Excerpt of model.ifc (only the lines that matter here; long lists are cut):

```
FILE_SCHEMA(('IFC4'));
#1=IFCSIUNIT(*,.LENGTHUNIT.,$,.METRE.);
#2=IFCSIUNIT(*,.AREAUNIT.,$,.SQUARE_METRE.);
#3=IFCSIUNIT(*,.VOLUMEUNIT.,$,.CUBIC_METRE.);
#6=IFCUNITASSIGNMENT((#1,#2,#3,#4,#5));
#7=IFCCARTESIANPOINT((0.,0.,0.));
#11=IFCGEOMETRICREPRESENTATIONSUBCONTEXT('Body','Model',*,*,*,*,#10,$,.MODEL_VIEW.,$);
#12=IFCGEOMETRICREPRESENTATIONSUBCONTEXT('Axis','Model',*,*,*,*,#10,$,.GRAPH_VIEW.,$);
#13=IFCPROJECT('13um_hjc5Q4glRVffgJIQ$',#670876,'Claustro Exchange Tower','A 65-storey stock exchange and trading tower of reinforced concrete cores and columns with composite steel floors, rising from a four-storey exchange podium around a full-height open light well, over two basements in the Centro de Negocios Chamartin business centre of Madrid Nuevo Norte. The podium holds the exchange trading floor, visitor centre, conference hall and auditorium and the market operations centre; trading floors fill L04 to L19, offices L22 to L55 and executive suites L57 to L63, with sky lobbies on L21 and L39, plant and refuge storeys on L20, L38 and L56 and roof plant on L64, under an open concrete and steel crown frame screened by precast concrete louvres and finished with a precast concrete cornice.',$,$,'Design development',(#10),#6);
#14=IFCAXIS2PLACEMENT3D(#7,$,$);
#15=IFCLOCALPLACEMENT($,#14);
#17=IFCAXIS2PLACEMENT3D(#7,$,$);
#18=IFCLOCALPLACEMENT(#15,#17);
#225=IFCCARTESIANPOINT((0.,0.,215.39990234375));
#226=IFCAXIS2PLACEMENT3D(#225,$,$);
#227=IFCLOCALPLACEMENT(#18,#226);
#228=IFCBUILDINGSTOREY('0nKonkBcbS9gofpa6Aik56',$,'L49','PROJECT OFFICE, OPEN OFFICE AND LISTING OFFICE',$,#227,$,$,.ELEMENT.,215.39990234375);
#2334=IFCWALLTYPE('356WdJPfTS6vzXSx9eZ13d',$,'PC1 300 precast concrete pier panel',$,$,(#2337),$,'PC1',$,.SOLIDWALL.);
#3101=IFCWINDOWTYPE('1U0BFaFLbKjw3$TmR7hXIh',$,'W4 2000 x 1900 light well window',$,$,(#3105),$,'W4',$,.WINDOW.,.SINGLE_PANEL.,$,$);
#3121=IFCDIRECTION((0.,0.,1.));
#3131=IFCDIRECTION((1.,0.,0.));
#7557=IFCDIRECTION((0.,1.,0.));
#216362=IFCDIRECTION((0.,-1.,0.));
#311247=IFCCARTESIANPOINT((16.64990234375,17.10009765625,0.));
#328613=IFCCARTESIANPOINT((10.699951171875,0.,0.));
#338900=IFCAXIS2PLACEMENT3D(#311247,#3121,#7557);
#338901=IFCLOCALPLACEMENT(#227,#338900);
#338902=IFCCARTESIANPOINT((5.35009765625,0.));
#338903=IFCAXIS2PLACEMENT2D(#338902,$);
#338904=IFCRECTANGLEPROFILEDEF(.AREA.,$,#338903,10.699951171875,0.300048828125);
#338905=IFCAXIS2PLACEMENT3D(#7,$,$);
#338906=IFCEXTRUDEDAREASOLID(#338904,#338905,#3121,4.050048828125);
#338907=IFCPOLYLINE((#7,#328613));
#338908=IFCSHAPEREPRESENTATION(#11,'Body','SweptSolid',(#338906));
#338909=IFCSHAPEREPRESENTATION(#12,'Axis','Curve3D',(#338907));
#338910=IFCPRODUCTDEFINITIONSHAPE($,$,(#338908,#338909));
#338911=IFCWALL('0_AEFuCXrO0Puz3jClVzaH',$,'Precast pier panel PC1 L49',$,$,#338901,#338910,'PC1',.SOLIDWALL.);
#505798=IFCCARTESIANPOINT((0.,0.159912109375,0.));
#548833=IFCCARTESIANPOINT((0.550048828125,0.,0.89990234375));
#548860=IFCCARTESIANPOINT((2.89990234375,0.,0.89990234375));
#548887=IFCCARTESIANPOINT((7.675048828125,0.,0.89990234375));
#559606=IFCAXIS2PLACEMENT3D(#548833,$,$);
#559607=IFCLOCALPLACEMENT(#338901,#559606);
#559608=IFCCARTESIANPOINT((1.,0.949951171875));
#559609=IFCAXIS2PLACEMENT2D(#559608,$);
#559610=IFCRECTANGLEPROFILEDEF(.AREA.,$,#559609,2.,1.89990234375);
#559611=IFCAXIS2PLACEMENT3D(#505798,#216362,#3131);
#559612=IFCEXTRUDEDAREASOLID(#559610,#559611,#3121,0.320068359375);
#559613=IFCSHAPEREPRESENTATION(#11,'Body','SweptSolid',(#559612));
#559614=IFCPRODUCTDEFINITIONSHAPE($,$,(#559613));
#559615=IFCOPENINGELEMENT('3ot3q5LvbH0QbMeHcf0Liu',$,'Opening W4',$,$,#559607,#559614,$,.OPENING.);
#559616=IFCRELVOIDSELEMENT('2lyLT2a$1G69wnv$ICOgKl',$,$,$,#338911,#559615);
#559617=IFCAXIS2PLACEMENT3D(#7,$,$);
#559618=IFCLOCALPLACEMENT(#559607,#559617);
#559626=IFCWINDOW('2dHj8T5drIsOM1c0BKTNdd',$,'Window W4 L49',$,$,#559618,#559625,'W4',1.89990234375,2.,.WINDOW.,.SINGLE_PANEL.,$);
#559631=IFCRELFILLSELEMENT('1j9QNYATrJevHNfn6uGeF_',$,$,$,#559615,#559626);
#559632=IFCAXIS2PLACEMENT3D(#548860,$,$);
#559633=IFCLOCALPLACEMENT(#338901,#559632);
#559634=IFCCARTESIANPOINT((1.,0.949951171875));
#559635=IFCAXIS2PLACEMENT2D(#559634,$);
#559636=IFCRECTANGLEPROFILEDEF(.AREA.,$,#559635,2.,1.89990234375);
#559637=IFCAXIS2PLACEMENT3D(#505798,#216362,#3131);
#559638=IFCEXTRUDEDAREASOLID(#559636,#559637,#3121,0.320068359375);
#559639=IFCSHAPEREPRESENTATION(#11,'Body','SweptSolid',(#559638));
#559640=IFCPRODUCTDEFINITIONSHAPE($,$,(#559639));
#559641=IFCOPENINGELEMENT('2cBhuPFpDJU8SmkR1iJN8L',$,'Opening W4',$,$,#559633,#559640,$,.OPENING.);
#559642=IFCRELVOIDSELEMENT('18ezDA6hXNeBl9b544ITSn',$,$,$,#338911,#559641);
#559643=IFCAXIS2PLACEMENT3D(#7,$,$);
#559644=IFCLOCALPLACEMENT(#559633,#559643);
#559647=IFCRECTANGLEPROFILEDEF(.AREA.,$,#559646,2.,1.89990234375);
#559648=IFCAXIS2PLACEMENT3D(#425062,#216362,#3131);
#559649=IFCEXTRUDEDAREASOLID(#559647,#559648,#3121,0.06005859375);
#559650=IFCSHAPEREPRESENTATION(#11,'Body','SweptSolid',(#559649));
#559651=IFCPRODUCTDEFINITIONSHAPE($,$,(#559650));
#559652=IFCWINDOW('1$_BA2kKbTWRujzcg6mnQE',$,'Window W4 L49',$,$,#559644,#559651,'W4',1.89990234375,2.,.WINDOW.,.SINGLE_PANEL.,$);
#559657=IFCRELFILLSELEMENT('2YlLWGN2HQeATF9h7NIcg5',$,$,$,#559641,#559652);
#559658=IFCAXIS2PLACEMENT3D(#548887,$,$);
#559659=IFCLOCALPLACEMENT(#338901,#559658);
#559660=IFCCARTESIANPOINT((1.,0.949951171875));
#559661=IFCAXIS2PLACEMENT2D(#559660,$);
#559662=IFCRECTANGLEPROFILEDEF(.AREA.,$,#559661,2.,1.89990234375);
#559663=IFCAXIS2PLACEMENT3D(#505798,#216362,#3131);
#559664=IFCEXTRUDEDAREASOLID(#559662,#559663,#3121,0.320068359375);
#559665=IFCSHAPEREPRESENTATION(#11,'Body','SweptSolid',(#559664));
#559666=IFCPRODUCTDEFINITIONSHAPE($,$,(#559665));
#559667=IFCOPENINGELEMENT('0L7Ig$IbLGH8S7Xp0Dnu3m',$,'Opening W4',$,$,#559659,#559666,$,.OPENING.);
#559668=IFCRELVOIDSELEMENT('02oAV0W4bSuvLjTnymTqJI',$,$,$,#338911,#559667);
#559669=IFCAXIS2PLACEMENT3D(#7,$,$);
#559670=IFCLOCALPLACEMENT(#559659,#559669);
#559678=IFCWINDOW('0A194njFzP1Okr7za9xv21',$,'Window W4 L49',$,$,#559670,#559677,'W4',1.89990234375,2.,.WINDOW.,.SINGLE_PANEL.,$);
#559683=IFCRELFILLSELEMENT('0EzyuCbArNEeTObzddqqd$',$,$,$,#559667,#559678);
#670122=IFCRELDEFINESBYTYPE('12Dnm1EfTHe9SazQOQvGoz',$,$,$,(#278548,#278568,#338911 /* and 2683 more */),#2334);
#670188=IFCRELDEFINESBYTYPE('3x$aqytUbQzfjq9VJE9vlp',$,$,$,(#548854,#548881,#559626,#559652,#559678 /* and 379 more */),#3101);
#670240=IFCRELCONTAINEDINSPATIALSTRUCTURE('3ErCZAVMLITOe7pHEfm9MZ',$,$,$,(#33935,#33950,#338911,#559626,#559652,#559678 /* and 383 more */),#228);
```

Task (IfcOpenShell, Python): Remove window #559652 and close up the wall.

```python
import ifcopenshell
import ifcopenshell.api.feature
import ifcopenshell.api.root
import ifcopenshell.geom
import ifcopenshell.util.shape

model = ifcopenshell.open("model.ifc")
settings = ifcopenshell.geom.settings()


def volume(element):
    """Net volume in cubic metres, openings subtracted."""
    shape = ifcopenshell.geom.create_shape(settings, element)
    return ifcopenshell.util.shape.get_volume(shape.geometry)


window = model.by_id(559652)
opening = window.FillsVoids[0].RelatingOpeningElement
wall = opening.VoidsElements[0].RelatingBuildingElement
before = volume(wall)

ifcopenshell.api.root.remove_product(model, product=window)
ifcopenshell.api.feature.remove_feature(model, feature=opening)

after = volume(wall)

print(f"wall volume {before:.3f} -> {after:.3f} m3")

model.write("model_v2.ifc")
```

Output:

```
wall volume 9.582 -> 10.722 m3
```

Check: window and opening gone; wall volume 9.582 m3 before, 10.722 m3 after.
